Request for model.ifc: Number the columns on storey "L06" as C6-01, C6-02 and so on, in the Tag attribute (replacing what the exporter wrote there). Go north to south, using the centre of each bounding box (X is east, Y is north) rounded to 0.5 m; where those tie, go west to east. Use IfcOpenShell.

First a look at what the model holds.

```python
import ifcopenshell
import ifcopenshell.util.element
import ifcopenshell.util.placement

model = ifcopenshell.open("model.ifc")
print(model.schema)
storey = next(s for s in model.by_type("IfcBuildingStorey") if s.Name == "L06")
columns = [e for e in ifcopenshell.util.element.get_decomposition(storey) if e.is_a("IfcColumn")]
for e in sorted(columns, key=lambda e: e.id()):
    origin = ifcopenshell.util.placement.get_local_placement(e.ObjectPlacement)[:3, 3]
    print(e.id(), e.Tag, e.Name, origin.round(2) + 0.0, sep=" | ")
```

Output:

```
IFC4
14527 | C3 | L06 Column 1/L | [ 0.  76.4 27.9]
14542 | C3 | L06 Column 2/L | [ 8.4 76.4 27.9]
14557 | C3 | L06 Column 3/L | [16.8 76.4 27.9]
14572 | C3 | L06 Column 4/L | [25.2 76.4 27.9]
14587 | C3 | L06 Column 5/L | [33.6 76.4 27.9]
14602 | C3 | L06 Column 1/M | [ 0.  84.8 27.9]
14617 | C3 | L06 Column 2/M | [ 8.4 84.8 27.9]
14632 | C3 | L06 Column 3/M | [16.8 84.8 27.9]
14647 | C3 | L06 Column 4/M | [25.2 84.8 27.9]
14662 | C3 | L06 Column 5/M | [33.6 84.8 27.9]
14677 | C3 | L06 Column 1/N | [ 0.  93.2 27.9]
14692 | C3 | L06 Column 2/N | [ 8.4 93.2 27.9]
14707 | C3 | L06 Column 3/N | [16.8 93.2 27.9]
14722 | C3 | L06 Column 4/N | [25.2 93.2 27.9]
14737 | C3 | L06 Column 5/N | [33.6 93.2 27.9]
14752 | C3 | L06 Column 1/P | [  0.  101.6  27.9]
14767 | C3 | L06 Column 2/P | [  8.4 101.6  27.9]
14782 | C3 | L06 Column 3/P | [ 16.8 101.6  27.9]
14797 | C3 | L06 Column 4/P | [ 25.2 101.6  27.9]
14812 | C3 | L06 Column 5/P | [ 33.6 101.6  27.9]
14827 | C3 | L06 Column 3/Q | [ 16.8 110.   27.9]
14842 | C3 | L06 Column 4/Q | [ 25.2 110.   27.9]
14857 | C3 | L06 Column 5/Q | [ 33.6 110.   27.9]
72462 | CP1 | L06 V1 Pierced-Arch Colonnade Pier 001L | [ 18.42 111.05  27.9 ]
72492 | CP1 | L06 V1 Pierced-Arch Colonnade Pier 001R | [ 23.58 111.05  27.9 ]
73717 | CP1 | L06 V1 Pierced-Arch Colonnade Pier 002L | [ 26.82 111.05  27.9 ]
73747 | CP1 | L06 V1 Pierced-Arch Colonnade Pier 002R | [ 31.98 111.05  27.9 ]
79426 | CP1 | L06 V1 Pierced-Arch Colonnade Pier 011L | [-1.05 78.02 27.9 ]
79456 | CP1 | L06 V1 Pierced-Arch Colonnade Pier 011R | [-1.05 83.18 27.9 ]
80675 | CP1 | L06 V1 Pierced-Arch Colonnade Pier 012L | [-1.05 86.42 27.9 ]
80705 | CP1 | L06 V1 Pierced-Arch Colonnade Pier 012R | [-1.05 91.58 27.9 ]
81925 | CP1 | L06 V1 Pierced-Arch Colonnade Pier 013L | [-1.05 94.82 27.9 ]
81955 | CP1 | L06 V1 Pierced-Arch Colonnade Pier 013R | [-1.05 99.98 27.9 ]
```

```python
import ifcopenshell
import ifcopenshell.geom
import ifcopenshell.util.element
import ifcopenshell.util.shape

model = ifcopenshell.open("model.ifc")
settings = ifcopenshell.geom.settings()
settings.set("use-world-coords", True)


def centre(element):
    shape = ifcopenshell.geom.create_shape(settings, element)
    return ifcopenshell.util.shape.get_bbox_centroid(shape.geometry)


storey = next(s for s in model.by_type("IfcBuildingStorey") if s.Name == "L06")
columns = [e for e in ifcopenshell.util.element.get_decomposition(storey) if e.is_a("IfcColumn")]

# Insertion points can sit at a corner or the storey origin, so sort by the geometry (in metres).
centres = {e: centre(e) for e in columns}
columns.sort(key=lambda e: (-round(centres[e][1] / 0.5), centres[e][0]))

for i, e in enumerate(columns, start=1):
    number = f"C6-{i:02d}"
    e.Tag = number
    print(e.id(), number)

model.write("model_rev.ifc")
```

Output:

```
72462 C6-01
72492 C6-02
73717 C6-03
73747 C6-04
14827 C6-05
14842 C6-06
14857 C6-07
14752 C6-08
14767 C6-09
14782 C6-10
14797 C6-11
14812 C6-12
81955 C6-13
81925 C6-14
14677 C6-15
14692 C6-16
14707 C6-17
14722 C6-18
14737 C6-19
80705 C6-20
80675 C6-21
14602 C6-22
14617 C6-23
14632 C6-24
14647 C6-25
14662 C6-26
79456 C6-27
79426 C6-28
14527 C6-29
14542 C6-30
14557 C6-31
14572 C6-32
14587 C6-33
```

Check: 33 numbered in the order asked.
